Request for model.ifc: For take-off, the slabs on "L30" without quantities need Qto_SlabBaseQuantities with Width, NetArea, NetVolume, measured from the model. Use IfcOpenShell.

First a look at what the model holds.

```python
import ifcopenshell
import ifcopenshell.util.element
import ifcopenshell.util.unit

model = ifcopenshell.open("model.ifc")
print(model.schema)
for unit_type in ("LENGTHUNIT", "AREAUNIT", "VOLUMEUNIT"):
    print(unit_type, ifcopenshell.util.unit.calculate_unit_scale(model, unit_type))
storey = next(s for s in model.by_type("IfcBuildingStorey") if s.Name == "L30")
slabs = [e for e in ifcopenshell.util.element.get_decomposition(storey) if e.is_a("IfcSlab")]
for e in sorted(slabs, key=lambda e: e.id()):
    print(e.id(), e.is_a(), e.Name, list(ifcopenshell.util.element.get_psets(e, qtos_only=True)), sep=" | ")
```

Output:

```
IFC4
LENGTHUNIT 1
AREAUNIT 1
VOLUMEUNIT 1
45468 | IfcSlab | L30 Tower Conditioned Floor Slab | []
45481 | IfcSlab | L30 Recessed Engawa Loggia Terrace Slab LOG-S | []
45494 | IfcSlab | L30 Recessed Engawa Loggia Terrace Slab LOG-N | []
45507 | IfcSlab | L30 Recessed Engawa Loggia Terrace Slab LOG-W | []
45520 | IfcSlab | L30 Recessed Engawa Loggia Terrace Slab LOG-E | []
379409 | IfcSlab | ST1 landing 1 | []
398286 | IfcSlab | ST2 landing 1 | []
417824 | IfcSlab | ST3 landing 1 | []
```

```python
import ifcopenshell
import ifcopenshell.api.pset
import ifcopenshell.geom
import ifcopenshell.util.element
import ifcopenshell.util.shape
import ifcopenshell.util.unit

model = ifcopenshell.open("model.ifc")
unit_scale = ifcopenshell.util.unit.calculate_unit_scale(model)
area_scale = ifcopenshell.util.unit.calculate_unit_scale(model, "AREAUNIT")
volume_scale = ifcopenshell.util.unit.calculate_unit_scale(model, "VOLUMEUNIT")
settings = ifcopenshell.geom.settings()

storey = next(s for s in model.by_type("IfcBuildingStorey") if s.Name == "L30")
slabs = [e for e in ifcopenshell.util.element.get_decomposition(storey) if e.is_a("IfcSlab")]

for e in sorted(slabs, key=lambda e: e.id()):
    if ifcopenshell.util.element.get_psets(e, qtos_only=True, should_inherit=False):
        continue
    # Geometry comes back in metres, in the element's own axes.
    shape = ifcopenshell.geom.create_shape(settings, e)
    values = {
        "Width": ifcopenshell.util.shape.get_z(shape.geometry) / unit_scale,
        "NetArea": ifcopenshell.util.shape.get_footprint_area(shape.geometry) / area_scale,
        "NetVolume": ifcopenshell.util.shape.get_volume(shape.geometry) / volume_scale,
    }
    qto = ifcopenshell.api.pset.add_qto(model, product=e, name="Qto_SlabBaseQuantities")
    ifcopenshell.api.pset.edit_qto(model, qto=qto, properties=values)
    print(e.id(), {k: round(v, 3) for k, v in values.items()})

model.write("model_updated.ifc")
```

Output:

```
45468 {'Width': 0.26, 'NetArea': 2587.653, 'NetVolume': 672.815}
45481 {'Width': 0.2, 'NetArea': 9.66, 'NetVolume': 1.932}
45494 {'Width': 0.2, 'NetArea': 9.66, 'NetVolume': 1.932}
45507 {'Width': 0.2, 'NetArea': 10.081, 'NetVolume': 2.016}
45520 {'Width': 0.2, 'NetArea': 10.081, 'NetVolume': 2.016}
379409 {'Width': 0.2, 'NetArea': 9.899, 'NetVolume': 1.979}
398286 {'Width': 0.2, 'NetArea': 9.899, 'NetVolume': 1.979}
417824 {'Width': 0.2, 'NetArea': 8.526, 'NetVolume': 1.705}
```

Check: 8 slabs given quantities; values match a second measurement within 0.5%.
